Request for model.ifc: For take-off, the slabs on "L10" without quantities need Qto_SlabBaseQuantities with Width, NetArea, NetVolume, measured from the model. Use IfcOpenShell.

First a look at what the model holds.

```python
import ifcopenshell
import ifcopenshell.util.element
import ifcopenshell.util.unit

model = ifcopenshell.open("model.ifc")
print(model.schema)
for unit_type in ("LENGTHUNIT", "AREAUNIT", "VOLUMEUNIT"):
    print(unit_type, ifcopenshell.util.unit.calculate_unit_scale(model, unit_type))
storey = next(s for s in model.by_type("IfcBuildingStorey") if s.Name == "L10")
slabs = [e for e in ifcopenshell.util.element.get_decomposition(storey) if e.is_a("IfcSlab")]
for e in sorted(slabs, key=lambda e: e.id()):
    print(e.id(), e.is_a(), e.Name, list(ifcopenshell.util.element.get_psets(e, qtos_only=True)), sep=" | ")
```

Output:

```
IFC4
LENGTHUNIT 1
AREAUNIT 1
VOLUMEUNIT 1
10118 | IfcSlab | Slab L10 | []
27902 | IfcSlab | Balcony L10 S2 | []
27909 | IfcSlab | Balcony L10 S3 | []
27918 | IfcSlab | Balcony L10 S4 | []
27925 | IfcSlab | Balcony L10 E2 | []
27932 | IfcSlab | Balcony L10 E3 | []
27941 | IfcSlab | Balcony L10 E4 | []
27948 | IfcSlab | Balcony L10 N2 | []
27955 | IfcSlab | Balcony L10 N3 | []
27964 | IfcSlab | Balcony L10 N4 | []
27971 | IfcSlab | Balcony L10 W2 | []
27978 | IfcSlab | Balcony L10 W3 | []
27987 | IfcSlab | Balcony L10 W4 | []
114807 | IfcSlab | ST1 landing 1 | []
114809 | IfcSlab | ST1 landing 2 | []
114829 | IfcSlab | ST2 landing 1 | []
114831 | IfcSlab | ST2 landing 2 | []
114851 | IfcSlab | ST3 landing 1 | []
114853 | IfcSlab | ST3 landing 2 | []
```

```python
import ifcopenshell
import ifcopenshell.api.pset
import ifcopenshell.geom
import ifcopenshell.util.element
import ifcopenshell.util.shape
import ifcopenshell.util.unit

model = ifcopenshell.open("model.ifc")
unit_scale = ifcopenshell.util.unit.calculate_unit_scale(model)
area_scale = ifcopenshell.util.unit.calculate_unit_scale(model, "AREAUNIT")
volume_scale = ifcopenshell.util.unit.calculate_unit_scale(model, "VOLUMEUNIT")
settings = ifcopenshell.geom.settings()

storey = next(s for s in model.by_type("IfcBuildingStorey") if s.Name == "L10")
slabs = [e for e in ifcopenshell.util.element.get_decomposition(storey) if e.is_a("IfcSlab")]

for e in sorted(slabs, key=lambda e: e.id()):
    if ifcopenshell.util.element.get_psets(e, qtos_only=True, should_inherit=False):
        continue
    # Geometry comes back in metres, in the element's own axes.
    shape = ifcopenshell.geom.create_shape(settings, e)
    values = {
        "Width": ifcopenshell.util.shape.get_z(shape.geometry) / unit_scale,
        "NetArea": ifcopenshell.util.shape.get_footprint_area(shape.geometry) / area_scale,
        "NetVolume": ifcopenshell.util.shape.get_volume(shape.geometry) / volume_scale,
    }
    qto = ifcopenshell.api.pset.add_qto(model, product=e, name="Qto_SlabBaseQuantities")
    ifcopenshell.api.pset.edit_qto(model, qto=qto, properties=values)
    print(e.id(), {k: round(v, 3) for k, v in values.items()})

model.write("model_rev.ifc")
```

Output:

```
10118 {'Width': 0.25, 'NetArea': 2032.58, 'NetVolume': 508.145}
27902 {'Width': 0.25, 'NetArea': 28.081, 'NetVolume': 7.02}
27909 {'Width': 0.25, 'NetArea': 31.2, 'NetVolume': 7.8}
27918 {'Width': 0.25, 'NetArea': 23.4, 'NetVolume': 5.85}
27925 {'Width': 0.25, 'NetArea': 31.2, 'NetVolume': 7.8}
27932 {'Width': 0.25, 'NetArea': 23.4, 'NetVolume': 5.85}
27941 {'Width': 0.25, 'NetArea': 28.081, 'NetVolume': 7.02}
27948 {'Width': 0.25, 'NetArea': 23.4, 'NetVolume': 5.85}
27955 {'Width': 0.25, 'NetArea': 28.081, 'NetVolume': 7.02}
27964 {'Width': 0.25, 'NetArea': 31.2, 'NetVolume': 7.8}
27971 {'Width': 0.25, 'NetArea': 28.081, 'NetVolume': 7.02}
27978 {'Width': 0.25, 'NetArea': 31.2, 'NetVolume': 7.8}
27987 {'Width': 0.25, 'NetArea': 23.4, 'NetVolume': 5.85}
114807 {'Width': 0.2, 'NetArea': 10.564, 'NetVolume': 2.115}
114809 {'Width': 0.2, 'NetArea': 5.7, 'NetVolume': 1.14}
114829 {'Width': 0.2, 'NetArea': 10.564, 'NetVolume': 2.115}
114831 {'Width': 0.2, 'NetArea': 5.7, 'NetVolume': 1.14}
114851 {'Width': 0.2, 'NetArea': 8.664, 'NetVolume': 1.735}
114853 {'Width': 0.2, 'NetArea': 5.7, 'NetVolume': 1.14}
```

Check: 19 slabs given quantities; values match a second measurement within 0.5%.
